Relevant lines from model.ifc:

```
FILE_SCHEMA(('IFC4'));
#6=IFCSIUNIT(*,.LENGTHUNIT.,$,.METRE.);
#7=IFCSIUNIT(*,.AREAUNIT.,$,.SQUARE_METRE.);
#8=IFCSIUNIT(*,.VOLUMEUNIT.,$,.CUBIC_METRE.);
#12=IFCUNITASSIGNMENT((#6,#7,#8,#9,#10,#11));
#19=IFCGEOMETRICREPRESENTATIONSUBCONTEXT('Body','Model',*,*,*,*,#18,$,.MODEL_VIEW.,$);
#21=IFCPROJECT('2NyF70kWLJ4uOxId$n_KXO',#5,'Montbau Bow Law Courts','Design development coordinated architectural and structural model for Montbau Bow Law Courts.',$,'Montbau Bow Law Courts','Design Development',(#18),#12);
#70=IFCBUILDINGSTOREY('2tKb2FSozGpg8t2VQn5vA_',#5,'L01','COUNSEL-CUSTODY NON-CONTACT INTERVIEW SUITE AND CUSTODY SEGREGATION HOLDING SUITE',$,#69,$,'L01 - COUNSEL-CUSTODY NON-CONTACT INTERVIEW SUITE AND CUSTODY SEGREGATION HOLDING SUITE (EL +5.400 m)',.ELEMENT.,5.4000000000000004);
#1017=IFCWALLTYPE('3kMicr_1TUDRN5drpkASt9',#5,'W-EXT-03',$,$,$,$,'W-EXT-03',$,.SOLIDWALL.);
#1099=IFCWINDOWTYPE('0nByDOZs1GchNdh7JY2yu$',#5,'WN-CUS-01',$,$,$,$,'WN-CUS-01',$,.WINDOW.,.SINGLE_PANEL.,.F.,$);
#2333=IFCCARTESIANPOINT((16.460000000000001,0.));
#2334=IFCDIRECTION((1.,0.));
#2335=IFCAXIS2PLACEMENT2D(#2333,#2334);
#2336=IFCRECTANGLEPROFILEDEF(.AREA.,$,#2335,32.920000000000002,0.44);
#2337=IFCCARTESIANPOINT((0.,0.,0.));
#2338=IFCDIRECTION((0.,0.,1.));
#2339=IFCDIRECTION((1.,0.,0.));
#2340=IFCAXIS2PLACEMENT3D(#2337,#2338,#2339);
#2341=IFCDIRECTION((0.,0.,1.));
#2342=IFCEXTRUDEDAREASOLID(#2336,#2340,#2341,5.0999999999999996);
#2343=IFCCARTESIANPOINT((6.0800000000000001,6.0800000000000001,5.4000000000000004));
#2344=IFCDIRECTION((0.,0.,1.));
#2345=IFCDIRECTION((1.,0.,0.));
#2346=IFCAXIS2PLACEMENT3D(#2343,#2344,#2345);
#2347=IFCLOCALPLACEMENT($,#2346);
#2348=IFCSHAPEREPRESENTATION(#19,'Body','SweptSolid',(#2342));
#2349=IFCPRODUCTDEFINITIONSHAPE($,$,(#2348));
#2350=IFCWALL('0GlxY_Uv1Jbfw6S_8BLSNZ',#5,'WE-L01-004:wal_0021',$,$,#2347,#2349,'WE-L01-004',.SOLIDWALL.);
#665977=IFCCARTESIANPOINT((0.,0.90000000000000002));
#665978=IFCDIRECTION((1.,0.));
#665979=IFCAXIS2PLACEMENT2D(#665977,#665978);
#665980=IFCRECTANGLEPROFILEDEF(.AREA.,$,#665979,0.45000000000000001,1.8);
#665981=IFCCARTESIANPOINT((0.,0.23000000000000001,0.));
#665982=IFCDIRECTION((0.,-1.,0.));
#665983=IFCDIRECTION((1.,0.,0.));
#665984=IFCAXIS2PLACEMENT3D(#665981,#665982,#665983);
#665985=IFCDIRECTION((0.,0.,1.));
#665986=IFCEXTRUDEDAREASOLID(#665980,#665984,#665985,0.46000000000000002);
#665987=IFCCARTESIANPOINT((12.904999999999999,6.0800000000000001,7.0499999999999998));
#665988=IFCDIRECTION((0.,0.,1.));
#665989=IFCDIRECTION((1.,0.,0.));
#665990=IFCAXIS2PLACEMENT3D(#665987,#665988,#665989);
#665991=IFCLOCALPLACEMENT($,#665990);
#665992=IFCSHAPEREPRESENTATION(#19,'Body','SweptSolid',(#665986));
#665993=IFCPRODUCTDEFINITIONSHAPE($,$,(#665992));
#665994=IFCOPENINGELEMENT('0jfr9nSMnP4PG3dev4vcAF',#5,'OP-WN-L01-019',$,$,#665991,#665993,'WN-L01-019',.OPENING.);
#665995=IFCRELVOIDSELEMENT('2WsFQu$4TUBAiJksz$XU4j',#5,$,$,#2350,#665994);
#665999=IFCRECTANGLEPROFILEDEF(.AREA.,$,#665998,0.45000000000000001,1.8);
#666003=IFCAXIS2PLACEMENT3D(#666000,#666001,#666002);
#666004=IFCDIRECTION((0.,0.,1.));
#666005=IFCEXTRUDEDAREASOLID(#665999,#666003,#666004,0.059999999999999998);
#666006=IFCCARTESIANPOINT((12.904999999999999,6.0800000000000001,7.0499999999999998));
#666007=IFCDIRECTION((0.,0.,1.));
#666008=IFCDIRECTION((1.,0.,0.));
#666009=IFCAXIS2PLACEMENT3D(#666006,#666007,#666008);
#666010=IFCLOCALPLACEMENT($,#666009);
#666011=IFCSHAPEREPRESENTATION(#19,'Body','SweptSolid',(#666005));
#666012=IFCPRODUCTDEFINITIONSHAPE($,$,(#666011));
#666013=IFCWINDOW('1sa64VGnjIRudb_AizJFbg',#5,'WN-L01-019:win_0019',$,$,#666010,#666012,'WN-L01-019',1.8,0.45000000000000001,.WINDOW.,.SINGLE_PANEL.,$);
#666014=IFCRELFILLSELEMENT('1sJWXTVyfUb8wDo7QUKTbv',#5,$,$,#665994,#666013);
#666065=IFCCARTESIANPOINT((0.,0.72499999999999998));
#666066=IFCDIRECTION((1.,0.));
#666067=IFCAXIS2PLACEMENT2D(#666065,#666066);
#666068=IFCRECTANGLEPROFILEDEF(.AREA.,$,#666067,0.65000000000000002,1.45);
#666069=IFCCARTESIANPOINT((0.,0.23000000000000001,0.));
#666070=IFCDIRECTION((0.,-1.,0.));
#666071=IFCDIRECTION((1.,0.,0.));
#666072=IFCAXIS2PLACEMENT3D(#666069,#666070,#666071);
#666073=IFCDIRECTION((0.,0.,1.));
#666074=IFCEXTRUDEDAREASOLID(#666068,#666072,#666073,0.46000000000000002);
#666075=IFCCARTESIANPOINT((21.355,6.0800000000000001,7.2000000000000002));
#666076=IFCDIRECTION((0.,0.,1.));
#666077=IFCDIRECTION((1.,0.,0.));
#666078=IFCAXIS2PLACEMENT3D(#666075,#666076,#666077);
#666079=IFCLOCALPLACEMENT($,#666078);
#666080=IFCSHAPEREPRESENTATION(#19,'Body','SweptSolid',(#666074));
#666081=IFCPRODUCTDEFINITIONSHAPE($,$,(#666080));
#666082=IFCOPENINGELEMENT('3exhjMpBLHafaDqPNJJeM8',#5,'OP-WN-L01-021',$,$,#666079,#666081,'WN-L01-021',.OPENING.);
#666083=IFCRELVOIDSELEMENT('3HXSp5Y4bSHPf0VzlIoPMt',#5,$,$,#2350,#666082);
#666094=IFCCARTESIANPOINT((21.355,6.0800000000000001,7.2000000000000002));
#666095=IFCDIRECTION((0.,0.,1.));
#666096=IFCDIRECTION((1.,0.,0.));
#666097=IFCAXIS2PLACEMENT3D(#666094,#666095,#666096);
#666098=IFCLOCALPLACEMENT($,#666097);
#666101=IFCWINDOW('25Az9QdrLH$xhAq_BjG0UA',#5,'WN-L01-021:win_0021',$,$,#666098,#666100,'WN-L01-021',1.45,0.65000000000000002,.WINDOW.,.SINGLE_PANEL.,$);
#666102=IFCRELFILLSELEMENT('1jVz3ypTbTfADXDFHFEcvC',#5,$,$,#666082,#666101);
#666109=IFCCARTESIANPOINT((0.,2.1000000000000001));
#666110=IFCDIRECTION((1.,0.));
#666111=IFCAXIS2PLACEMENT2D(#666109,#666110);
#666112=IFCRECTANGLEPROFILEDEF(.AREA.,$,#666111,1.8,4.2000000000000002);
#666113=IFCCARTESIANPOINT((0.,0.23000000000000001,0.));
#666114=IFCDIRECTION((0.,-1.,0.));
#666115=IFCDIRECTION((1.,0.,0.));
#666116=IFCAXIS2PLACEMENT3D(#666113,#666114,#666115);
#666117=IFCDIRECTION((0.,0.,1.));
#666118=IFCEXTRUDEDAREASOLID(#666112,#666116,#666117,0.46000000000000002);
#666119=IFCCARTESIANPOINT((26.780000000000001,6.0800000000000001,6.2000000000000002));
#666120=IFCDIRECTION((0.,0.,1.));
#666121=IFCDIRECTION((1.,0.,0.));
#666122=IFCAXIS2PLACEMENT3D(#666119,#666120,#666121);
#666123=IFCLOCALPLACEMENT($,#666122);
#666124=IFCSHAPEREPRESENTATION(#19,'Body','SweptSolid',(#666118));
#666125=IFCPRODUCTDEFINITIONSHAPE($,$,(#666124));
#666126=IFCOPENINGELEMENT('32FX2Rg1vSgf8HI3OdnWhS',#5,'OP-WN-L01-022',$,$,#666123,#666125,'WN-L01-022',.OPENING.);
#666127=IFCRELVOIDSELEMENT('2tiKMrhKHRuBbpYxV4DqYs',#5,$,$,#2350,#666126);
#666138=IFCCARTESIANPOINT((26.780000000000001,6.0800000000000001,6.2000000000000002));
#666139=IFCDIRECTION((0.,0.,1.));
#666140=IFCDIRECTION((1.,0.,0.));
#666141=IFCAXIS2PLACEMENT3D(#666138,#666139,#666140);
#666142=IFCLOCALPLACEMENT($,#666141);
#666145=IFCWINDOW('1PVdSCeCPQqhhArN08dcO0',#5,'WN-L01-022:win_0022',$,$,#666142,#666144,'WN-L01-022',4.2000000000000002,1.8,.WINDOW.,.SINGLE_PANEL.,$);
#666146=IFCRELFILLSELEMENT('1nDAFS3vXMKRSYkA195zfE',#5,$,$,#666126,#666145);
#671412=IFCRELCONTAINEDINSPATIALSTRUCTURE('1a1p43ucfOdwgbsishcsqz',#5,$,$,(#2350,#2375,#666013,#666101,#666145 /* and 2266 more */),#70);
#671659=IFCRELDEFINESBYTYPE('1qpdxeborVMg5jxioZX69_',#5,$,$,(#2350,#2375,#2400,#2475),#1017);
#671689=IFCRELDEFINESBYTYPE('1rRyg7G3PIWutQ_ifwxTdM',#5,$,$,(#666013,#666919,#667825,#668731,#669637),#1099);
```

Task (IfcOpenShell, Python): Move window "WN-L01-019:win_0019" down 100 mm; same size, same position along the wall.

```python
import numpy as np
import ifcopenshell
import ifcopenshell.api.geometry
import ifcopenshell.util.placement
import ifcopenshell.util.unit

model = ifcopenshell.open("model.ifc")
unit_scale = ifcopenshell.util.unit.calculate_unit_scale(model)

window = model.by_guid("1sa64VGnjIRudb_AizJFbg")
opening = window.FillsVoids[0].RelatingOpeningElement
dz = -0.1

shift = np.array([0.0, 0.0, dz])
# The window is not placed relative to its opening, so move both.
for product in (opening, window):
    matrix = ifcopenshell.util.placement.get_local_placement(product.ObjectPlacement)
    matrix[:3, 3] += shift
    ifcopenshell.api.geometry.edit_object_placement(model, product=product, matrix=matrix, is_si=False)

print(f"moved by {dz * unit_scale:+.3f} m")

model.write("model_updated.ifc")
```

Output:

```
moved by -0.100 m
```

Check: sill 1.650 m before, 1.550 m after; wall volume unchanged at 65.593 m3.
